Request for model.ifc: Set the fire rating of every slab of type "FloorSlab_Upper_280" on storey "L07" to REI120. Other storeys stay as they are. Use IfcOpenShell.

First a look at what the model holds.

```python
import ifcopenshell
import ifcopenshell.util.element

model = ifcopenshell.open("model.ifc")
print(model.schema)
storey = next(s for s in model.by_type("IfcBuildingStorey") if s.Name == "L07")
slabs = [e for e in ifcopenshell.util.element.get_decomposition(storey) if e.is_a("IfcSlab")]
seen = {}
for e in slabs:
    element_type = ifcopenshell.util.element.get_type(e)
    key = (element_type.Name if element_type != e and element_type else None, ifcopenshell.util.element.get_pset(e, "Pset_SlabCommon", "FireRating"))
    seen[key] = seen.get(key, 0) + 1
for (name, value), count in sorted(seen.items(), key=str):
    print(count, "x", name, "|", value)
```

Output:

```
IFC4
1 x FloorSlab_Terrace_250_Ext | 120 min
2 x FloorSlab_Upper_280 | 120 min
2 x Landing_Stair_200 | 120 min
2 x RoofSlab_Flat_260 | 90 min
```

```python
import ifcopenshell
import ifcopenshell.api.pset
import ifcopenshell.util.element

model = ifcopenshell.open("model.ifc")

storey = next(s for s in model.by_type("IfcBuildingStorey") if s.Name == "L07")
slabs = [e for e in ifcopenshell.util.element.get_decomposition(storey) if e.is_a("IfcSlab")]

count = 0
for e in slabs:
    element_type = ifcopenshell.util.element.get_type(e)
    if element_type in (None, e) or element_type.Name != "FloorSlab_Upper_280":
        continue
    # add_pset returns the element's existing set when there is one.
    pset = ifcopenshell.api.pset.add_pset(model, product=e, name="Pset_SlabCommon")
    ifcopenshell.api.pset.edit_pset(model, pset=pset, properties={"FireRating": "REI120"})
    count += 1

print(count, "slabs updated")

model.write("model_edited.ifc")
```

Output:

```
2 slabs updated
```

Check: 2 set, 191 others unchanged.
